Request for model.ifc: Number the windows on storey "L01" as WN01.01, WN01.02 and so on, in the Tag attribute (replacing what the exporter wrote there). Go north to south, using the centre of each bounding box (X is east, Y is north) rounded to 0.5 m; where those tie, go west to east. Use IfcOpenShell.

First a look at what the model holds.

```python
import ifcopenshell
import ifcopenshell.util.element
import ifcopenshell.util.placement

model = ifcopenshell.open("model.ifc")
print(model.schema)
storey = next(s for s in model.by_type("IfcBuildingStorey") if s.Name == "L01")
windows = [e for e in ifcopenshell.util.element.get_decomposition(storey) if e.is_a("IfcWindow")]
for e in sorted(windows, key=lambda e: e.id()):
    origin = ifcopenshell.util.placement.get_local_placement(e.ObjectPlacement)[:3, 3]
    print(e.id(), e.Tag, e.Name, origin.round(2) + 0.0, sep=" | ")
```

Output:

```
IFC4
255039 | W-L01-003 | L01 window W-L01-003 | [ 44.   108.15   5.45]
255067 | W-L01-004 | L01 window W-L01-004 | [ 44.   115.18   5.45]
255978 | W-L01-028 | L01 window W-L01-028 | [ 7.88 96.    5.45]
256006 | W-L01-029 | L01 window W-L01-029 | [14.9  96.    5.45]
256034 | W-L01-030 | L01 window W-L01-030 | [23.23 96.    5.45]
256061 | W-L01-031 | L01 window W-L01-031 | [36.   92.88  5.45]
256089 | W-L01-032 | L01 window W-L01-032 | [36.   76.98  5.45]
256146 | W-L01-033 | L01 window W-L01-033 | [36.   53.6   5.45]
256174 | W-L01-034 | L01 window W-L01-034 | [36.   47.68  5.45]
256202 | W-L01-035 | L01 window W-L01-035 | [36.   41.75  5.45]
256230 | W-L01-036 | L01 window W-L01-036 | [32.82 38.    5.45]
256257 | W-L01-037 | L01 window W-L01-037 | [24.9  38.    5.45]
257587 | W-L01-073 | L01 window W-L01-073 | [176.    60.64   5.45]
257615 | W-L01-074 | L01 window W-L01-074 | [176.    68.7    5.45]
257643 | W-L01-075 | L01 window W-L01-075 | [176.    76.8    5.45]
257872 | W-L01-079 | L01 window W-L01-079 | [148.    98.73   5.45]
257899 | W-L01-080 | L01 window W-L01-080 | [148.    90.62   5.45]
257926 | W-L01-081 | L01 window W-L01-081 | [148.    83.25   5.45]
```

```python
import ifcopenshell
import ifcopenshell.geom
import ifcopenshell.util.element
import ifcopenshell.util.shape

model = ifcopenshell.open("model.ifc")
settings = ifcopenshell.geom.settings()
settings.set("use-world-coords", True)


def centre(element):
    shape = ifcopenshell.geom.create_shape(settings, element)
    return ifcopenshell.util.shape.get_bbox_centroid(shape.geometry)


storey = next(s for s in model.by_type("IfcBuildingStorey") if s.Name == "L01")
windows = [e for e in ifcopenshell.util.element.get_decomposition(storey) if e.is_a("IfcWindow")]

# Insertion points can sit at a corner or the storey origin, so sort by the geometry (in metres).
centres = {e: centre(e) for e in windows}
windows.sort(key=lambda e: (-round(centres[e][1] / 0.5), centres[e][0]))

for i, e in enumerate(windows, start=1):
    number = f"WN01.{i:02d}"
    e.Tag = number
    print(e.id(), number)

model.write("model_edited.ifc")
```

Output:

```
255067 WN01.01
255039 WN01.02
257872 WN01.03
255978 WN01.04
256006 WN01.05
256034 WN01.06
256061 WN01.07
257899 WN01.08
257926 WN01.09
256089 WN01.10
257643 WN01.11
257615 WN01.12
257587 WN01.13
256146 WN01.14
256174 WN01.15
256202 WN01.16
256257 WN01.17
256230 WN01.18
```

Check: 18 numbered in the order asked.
